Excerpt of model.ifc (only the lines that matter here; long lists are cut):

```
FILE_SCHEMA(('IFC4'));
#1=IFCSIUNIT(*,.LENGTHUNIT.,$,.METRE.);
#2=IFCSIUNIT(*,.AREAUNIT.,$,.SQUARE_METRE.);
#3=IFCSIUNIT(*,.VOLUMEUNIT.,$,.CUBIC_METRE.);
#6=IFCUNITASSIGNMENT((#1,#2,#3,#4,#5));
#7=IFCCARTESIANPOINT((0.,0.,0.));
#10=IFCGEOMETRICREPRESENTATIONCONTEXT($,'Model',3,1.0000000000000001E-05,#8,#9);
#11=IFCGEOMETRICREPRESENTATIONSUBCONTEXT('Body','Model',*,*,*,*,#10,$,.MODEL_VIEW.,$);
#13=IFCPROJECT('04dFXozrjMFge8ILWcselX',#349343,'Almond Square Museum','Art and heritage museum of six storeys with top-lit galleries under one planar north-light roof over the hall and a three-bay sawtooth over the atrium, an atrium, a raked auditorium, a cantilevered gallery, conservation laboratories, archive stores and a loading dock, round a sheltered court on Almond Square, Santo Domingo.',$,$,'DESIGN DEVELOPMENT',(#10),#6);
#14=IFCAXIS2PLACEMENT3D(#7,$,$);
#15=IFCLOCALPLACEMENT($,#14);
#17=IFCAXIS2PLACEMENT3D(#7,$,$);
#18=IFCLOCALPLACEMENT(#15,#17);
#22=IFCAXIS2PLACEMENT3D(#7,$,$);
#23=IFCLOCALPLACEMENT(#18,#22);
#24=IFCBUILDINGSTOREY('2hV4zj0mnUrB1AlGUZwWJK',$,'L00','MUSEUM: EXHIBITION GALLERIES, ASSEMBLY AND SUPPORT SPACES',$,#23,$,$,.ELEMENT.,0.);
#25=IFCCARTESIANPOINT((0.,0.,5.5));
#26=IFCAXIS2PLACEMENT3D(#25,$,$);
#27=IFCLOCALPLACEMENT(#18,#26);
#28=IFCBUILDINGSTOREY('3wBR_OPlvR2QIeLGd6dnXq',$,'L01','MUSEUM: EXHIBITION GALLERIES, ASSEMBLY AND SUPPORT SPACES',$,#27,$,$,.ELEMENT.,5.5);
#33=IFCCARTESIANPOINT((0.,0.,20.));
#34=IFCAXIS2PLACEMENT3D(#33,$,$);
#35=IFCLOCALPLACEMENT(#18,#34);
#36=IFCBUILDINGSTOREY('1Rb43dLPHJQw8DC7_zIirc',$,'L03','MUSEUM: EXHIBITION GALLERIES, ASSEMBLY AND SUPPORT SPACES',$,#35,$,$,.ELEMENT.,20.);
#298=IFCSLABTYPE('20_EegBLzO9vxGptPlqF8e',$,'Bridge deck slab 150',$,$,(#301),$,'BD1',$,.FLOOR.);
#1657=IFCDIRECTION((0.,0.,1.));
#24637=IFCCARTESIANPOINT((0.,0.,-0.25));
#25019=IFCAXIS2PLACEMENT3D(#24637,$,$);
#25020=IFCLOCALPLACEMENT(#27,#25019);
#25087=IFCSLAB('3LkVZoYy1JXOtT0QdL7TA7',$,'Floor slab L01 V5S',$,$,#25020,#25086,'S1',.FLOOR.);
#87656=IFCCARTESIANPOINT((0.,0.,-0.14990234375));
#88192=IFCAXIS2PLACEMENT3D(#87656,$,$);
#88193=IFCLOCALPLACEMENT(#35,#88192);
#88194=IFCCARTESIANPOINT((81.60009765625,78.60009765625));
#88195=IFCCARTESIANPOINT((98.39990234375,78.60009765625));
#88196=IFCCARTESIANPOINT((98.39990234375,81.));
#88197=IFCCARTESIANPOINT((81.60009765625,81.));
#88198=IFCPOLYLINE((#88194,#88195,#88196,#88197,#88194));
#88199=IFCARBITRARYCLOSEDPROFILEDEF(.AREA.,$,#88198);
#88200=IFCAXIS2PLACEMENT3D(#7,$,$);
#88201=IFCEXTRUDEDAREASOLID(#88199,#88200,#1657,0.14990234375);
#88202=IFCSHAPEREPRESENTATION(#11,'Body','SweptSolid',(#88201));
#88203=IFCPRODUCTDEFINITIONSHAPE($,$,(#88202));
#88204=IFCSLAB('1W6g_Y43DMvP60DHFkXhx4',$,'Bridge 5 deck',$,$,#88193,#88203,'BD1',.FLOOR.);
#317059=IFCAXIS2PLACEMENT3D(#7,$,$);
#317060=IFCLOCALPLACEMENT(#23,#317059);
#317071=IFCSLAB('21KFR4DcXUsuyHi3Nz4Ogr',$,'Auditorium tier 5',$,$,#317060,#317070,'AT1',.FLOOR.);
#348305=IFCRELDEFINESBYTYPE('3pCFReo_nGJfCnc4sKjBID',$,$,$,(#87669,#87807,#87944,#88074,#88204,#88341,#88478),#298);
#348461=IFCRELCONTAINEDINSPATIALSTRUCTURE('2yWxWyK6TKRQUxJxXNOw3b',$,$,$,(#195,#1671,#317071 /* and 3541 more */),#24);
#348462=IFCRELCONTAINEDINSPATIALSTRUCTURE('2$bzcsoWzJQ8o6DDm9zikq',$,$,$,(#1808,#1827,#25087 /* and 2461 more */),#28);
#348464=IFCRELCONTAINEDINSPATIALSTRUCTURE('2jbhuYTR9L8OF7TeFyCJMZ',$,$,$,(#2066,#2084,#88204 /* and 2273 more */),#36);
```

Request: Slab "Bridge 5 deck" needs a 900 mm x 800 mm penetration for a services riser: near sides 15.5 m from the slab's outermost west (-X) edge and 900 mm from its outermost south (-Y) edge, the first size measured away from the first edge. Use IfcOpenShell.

```python
import numpy as np
import ifcopenshell
import ifcopenshell.api.feature
import ifcopenshell.api.geometry
import ifcopenshell.api.root
import ifcopenshell.geom
import ifcopenshell.util.placement
import ifcopenshell.util.representation
import ifcopenshell.util.shape
import ifcopenshell.util.unit

model = ifcopenshell.open("model.ifc")
unit_scale = ifcopenshell.util.unit.calculate_unit_scale(model)
settings = ifcopenshell.geom.settings()


def volume(element):
    """Net volume in cubic metres, openings subtracted."""
    shape = ifcopenshell.geom.create_shape(settings, element)
    return ifcopenshell.util.shape.get_volume(shape.geometry)


slab = model.by_id(88204)
before = volume(slab)

# Extent in the slab's own axes, in metres. The edges named are its -X and -Y sides.
slab_shape = ifcopenshell.geom.create_shape(settings, slab)
vertices = ifcopenshell.util.shape.get_vertices(slab_shape.geometry)
x_min, y_min, bottom = vertices.min(axis=0)
top = vertices[:, 2].max()

opening = ifcopenshell.api.root.create_entity(model, ifc_class="IfcOpeningElement", name="Services riser opening", predefined_type="OPENING")
context = ifcopenshell.util.representation.get_context(model, "Model", "Body", "MODEL_VIEW")
width, depth = 0.9, 0.8
outline = [(0.0, 0.0), (width, 0.0), (width, depth), (0.0, depth), (0.0, 0.0)]
# Overshoot both faces by 50 mm so the cut is clean.
shape = ifcopenshell.api.geometry.add_slab_representation(
    model, context=context, depth=top - bottom + 0.1, polyline=outline
)
ifcopenshell.api.geometry.assign_representation(model, product=opening, representation=shape)

matrix = ifcopenshell.util.placement.get_local_placement(slab.ObjectPlacement)
matrix[:, 3] = matrix @ np.append(np.array([x_min + 15.5, y_min + 0.9, bottom - 0.05]) / unit_scale, 1.0)
ifcopenshell.api.geometry.edit_object_placement(model, product=opening, matrix=matrix, is_si=False)
ifcopenshell.api.feature.add_feature(model, feature=opening, element=slab)

after = volume(slab)

print(f"slab volume {before:.3f} -> {after:.3f} m3")

model.write("model_rev.ifc")
```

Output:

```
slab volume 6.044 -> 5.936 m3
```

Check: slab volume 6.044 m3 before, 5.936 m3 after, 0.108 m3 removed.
